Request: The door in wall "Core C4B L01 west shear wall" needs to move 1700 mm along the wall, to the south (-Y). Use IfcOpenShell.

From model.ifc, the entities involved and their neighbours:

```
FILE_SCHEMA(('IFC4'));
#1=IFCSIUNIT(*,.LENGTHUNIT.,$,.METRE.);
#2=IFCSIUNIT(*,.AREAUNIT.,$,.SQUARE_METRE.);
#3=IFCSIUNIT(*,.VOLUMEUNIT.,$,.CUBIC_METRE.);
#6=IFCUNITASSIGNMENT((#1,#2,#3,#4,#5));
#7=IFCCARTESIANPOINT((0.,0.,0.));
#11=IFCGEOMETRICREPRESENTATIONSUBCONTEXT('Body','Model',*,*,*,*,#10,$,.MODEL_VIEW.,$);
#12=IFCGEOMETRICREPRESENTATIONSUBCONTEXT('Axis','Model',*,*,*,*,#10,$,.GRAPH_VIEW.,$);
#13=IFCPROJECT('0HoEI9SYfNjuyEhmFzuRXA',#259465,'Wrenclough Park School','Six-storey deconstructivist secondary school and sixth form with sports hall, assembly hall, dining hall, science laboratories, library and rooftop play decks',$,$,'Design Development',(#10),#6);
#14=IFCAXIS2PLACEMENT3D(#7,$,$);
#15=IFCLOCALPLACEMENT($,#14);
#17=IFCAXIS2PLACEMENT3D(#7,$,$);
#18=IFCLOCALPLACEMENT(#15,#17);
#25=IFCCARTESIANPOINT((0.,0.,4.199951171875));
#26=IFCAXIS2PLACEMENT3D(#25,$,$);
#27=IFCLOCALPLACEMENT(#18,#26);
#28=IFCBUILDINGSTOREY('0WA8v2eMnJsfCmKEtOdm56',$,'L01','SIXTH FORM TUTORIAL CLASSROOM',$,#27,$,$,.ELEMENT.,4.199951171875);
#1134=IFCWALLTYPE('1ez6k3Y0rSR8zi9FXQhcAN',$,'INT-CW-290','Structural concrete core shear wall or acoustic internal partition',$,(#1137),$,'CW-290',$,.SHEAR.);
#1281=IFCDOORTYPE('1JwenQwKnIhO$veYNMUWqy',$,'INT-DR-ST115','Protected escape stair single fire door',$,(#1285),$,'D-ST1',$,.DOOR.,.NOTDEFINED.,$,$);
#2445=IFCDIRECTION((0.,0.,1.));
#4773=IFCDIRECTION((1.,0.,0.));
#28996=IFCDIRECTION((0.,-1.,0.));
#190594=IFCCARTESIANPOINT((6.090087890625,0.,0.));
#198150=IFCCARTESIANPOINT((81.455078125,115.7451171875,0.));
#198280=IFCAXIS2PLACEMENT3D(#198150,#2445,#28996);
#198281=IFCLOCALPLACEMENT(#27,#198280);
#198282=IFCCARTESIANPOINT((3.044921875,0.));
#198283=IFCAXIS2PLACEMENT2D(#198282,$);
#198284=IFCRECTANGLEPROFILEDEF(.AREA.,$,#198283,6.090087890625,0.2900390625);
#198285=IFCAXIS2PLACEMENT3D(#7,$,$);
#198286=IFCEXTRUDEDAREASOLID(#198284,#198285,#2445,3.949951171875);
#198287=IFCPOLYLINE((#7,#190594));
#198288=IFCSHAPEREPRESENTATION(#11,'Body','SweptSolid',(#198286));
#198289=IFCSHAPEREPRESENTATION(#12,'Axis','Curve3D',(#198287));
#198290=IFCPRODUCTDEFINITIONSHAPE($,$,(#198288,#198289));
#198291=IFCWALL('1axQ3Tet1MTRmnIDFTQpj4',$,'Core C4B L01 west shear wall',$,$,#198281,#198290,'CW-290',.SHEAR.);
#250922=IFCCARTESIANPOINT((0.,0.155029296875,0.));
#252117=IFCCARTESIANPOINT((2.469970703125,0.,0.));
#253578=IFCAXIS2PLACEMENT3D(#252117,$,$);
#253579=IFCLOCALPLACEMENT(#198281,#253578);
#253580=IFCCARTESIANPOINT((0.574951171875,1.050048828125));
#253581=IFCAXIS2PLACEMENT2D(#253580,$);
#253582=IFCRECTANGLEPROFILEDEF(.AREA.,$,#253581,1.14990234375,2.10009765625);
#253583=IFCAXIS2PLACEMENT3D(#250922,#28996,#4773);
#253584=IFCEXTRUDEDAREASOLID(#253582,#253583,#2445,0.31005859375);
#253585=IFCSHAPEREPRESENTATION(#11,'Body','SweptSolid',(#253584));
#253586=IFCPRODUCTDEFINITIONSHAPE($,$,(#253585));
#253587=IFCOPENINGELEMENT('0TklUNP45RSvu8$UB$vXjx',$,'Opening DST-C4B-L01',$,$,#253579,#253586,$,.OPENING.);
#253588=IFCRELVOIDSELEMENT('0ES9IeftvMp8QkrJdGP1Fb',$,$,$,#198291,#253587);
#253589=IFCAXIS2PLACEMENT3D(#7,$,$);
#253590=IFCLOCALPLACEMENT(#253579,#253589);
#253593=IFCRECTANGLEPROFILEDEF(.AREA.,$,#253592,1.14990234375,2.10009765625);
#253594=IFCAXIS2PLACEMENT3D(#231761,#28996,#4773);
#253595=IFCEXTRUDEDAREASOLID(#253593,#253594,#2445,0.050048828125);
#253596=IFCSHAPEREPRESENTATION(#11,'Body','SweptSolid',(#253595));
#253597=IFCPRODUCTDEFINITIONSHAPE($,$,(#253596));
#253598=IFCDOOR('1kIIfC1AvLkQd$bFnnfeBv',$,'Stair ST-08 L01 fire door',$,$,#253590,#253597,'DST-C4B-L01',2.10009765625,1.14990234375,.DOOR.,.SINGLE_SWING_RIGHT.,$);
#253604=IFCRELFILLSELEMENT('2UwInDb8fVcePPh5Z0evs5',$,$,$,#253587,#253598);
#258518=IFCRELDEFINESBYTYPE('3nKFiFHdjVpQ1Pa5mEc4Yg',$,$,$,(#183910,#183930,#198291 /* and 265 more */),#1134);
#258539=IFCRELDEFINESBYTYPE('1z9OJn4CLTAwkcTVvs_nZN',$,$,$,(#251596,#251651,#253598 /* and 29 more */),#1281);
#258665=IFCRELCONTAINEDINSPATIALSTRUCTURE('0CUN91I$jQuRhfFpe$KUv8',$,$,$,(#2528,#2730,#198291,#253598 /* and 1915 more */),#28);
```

```python
import ifcopenshell
import ifcopenshell.api.geometry
import ifcopenshell.util.placement

model = ifcopenshell.open("model.ifc")

door = model.by_guid("1kIIfC1AvLkQd$bFnnfeBv")
opening = door.FillsVoids[0].RelatingOpeningElement
wall = opening.VoidsElements[0].RelatingBuildingElement

wall_matrix = ifcopenshell.util.placement.get_local_placement(wall.ObjectPlacement)
shift = wall_matrix[:3, 0] * 1.7
before = ifcopenshell.util.placement.get_local_placement(door.ObjectPlacement)[:3, 3].copy()

# The door is placed relative to its opening, so it follows when the opening moves.
matrix = ifcopenshell.util.placement.get_local_placement(opening.ObjectPlacement)
matrix[:3, 3] += shift
ifcopenshell.api.geometry.edit_object_placement(
    model, product=opening, matrix=matrix, is_si=False, should_transform_children=True
)

after = ifcopenshell.util.placement.get_local_placement(door.ObjectPlacement)[:3, 3]
print("door moved by", (after - before).round(3) + 0.0)

model.write("model_edited.ifc")
```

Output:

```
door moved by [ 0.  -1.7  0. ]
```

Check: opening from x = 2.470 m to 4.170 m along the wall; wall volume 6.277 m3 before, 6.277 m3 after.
